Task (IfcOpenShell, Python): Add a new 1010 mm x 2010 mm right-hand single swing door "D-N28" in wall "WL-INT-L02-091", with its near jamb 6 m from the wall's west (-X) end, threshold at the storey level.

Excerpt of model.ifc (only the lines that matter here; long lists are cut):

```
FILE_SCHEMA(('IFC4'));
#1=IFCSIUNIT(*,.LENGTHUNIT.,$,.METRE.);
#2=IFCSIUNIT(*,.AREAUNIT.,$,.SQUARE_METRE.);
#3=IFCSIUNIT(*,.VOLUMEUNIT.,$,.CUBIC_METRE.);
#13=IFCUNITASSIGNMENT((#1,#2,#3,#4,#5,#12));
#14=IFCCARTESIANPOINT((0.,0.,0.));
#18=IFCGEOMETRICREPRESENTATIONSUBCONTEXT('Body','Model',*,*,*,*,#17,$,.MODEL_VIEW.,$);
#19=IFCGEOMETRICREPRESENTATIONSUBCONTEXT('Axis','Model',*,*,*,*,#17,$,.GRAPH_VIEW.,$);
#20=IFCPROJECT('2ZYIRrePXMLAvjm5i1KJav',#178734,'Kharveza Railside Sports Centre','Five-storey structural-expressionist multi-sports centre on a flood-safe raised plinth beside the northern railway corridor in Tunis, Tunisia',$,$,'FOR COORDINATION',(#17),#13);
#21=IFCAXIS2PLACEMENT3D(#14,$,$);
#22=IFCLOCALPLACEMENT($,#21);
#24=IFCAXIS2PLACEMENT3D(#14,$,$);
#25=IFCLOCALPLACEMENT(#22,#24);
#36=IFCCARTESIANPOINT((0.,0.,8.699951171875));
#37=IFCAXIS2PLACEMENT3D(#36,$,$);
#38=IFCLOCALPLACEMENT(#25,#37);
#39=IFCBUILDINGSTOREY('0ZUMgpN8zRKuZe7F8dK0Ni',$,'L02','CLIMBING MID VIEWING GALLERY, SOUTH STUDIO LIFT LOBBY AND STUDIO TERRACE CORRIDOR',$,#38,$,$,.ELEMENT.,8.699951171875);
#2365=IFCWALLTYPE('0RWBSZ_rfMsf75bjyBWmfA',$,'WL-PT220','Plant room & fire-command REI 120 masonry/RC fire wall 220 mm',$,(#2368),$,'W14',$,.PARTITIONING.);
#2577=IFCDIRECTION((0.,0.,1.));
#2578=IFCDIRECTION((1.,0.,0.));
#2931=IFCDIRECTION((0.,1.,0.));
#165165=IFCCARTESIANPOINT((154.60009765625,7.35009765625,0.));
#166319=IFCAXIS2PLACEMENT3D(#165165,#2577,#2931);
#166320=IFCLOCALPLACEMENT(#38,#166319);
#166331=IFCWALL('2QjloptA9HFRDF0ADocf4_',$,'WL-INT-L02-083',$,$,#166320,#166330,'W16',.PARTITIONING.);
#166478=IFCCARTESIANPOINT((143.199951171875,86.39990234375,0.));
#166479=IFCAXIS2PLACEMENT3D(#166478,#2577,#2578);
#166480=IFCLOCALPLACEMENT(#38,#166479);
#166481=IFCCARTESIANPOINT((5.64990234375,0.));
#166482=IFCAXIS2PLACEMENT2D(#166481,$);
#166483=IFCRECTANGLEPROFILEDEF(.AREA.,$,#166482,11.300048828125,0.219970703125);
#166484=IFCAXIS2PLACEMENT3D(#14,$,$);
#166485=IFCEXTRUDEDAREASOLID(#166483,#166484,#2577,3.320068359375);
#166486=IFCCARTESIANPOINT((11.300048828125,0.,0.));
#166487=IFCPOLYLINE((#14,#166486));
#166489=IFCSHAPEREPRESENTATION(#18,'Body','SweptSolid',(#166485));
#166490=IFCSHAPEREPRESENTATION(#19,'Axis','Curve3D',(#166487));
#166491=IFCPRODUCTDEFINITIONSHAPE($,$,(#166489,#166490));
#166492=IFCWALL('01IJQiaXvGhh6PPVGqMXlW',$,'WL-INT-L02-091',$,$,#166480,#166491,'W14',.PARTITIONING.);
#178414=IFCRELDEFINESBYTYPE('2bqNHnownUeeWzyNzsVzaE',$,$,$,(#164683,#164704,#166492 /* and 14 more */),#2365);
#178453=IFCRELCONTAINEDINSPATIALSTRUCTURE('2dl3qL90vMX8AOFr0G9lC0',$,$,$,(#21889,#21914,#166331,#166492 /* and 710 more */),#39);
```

```python
import numpy as np
import ifcopenshell
import ifcopenshell.api.feature
import ifcopenshell.api.geometry
import ifcopenshell.api.root
import ifcopenshell.api.spatial
import ifcopenshell.geom
import ifcopenshell.util.element
import ifcopenshell.util.placement
import ifcopenshell.util.representation
import ifcopenshell.util.shape
import ifcopenshell.util.unit

model = ifcopenshell.open("model.ifc")
unit_scale = ifcopenshell.util.unit.calculate_unit_scale(model)
settings = ifcopenshell.geom.settings()


def volume(element):
    """Net volume in cubic metres, openings subtracted."""
    shape = ifcopenshell.geom.create_shape(settings, element)
    return ifcopenshell.util.shape.get_volume(shape.geometry)


wall = model.by_guid("01IJQiaXvGhh6PPVGqMXlW")
storey = ifcopenshell.util.element.get_container(wall, ifc_class="IfcBuildingStorey")
context = ifcopenshell.util.representation.get_context(model, "Model", "Body", "MODEL_VIEW")
before = volume(wall)

width, height, from_end, sill = 1.01, 2.01, 6, 0.0  # metres

# The wall runs along its own X axis, and the end named is its -X end.
wall_shape = ifcopenshell.geom.create_shape(settings, wall)
x, y, z = ifcopenshell.util.shape.get_vertices(wall_shape.geometry).T
start = x.min() + from_end
face, thickness = float(y.min()), float(y.max() - y.min())
wall_matrix = ifcopenshell.util.placement.get_local_placement(wall.ObjectPlacement)
level = ifcopenshell.util.placement.get_local_placement(storey.ObjectPlacement)[2, 3]


def in_wall(x, y):
    """Placement at x, y metres in the wall's axes, at sill height."""
    matrix = wall_matrix.copy()
    matrix[:, 3] = wall_matrix @ np.array([x / unit_scale, y / unit_scale, 0.0, 1.0])
    matrix[2, 3] = level + sill / unit_scale
    return matrix


# Opening: a box that overshoots both wall faces by 50 mm.
opening = ifcopenshell.api.root.create_entity(model, ifc_class="IfcOpeningElement", predefined_type="OPENING")
box = ifcopenshell.api.geometry.add_wall_representation(
    model, context=context, length=width, height=height, thickness=thickness + 0.1
)
ifcopenshell.api.geometry.assign_representation(model, product=opening, representation=box)
ifcopenshell.api.geometry.edit_object_placement(model, product=opening, matrix=in_wall(start, face - 0.05), is_si=False)
ifcopenshell.api.feature.add_feature(model, feature=opening, element=wall)

door = ifcopenshell.api.root.create_entity(model, ifc_class="IfcDoor", name="D-N28", predefined_type="DOOR")
door.OverallWidth, door.OverallHeight = width / unit_scale, height / unit_scale
door.OperationType = "SINGLE_SWING_RIGHT"
body = ifcopenshell.api.geometry.add_door_representation(
    model,
    context=context,
    overall_width=door.OverallWidth,
    overall_height=door.OverallHeight,
    operation_type="SINGLE_SWING_RIGHT",
    lining_properties={"LiningDepth": thickness / unit_scale, "ThresholdDepth": thickness / unit_scale},
)
ifcopenshell.api.geometry.assign_representation(model, product=door, representation=body)
ifcopenshell.api.spatial.assign_container(model, products=[door], relating_structure=storey)
ifcopenshell.api.feature.add_filling(model, opening=opening, element=door)

# The lining spans the wall, so the door starts at the wall face.
ifcopenshell.api.geometry.edit_object_placement(model, product=door, matrix=in_wall(start, face), is_si=False)

after = volume(wall)

print(f"wall volume {before:.3f} -> {after:.3f} m3")

model.write("model_v2.ifc")
```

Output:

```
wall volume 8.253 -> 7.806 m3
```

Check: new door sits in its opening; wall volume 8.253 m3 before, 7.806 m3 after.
